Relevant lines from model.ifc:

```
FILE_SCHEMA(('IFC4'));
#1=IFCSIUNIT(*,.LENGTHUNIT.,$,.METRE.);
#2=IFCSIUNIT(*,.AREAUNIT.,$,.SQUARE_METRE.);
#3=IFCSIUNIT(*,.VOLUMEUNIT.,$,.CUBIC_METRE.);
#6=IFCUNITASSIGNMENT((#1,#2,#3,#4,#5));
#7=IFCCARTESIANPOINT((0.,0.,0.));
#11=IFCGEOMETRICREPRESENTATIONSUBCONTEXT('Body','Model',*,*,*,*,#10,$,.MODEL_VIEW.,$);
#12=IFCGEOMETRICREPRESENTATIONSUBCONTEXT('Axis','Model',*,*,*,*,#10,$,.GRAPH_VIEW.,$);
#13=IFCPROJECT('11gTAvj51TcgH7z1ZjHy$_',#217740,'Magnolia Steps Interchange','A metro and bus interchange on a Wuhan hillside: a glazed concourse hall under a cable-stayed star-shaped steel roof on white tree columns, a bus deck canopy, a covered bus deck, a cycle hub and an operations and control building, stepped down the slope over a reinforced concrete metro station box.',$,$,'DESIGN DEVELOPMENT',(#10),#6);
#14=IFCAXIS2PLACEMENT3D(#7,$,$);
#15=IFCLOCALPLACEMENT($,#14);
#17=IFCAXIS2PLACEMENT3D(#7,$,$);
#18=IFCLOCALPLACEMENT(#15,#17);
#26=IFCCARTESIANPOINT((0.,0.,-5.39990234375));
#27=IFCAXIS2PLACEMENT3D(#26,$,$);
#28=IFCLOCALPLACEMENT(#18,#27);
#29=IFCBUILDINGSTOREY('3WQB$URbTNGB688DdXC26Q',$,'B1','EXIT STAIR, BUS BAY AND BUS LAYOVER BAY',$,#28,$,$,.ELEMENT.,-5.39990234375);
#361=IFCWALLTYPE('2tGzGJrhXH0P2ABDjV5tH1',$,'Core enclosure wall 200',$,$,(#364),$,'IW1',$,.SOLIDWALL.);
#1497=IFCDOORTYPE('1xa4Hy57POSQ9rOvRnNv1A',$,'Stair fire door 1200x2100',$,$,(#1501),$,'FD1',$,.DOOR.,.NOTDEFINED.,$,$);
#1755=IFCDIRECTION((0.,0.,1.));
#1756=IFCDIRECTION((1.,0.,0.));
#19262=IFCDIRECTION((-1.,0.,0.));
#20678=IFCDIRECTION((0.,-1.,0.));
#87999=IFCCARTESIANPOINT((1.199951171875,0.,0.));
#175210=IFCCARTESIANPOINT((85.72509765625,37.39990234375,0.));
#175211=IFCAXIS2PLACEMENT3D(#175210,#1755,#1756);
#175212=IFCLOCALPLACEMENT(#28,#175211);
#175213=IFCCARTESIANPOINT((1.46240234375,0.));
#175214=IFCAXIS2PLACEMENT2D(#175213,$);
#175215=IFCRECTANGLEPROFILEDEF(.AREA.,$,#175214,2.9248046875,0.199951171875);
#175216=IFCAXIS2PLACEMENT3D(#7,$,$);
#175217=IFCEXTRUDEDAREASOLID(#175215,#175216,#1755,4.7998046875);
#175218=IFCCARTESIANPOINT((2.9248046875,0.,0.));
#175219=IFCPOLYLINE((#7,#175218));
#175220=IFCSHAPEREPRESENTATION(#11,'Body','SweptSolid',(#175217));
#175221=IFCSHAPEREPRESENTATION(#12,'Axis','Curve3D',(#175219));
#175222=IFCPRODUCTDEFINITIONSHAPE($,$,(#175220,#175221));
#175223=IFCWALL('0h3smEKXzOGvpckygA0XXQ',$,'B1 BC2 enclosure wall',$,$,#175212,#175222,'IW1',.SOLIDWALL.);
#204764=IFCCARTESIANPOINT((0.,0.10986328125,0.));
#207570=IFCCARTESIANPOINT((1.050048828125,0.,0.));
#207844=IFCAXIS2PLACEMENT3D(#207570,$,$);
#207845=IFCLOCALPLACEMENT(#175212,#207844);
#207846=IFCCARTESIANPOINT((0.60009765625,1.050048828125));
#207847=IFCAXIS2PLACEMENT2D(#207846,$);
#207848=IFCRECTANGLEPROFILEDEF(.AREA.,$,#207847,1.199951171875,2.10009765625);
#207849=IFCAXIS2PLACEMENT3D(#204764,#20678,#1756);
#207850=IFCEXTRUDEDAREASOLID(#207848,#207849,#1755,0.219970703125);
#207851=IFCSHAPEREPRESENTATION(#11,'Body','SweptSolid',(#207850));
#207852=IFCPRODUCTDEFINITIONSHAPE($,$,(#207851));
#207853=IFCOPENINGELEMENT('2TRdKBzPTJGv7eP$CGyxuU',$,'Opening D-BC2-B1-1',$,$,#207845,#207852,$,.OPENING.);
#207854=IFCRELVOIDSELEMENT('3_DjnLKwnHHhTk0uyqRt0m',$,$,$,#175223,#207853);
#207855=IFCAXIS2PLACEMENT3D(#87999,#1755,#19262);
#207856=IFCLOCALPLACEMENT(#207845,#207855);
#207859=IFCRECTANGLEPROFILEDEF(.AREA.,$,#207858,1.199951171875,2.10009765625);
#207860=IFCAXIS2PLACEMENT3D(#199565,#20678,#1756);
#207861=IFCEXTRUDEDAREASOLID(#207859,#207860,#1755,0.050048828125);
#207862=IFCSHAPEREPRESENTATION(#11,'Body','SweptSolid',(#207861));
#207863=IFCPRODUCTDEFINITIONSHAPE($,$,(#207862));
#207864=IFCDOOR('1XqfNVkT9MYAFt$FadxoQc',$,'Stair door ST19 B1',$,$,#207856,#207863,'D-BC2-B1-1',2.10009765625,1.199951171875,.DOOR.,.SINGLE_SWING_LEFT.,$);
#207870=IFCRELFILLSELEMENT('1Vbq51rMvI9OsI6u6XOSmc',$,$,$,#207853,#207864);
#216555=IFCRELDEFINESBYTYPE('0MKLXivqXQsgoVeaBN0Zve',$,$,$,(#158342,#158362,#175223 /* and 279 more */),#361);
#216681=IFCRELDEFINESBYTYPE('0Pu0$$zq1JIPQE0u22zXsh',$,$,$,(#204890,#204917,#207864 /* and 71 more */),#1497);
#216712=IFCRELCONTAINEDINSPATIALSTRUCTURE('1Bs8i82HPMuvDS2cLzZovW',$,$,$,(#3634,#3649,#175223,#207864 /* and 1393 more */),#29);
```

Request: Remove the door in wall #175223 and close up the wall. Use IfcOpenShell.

```python
import ifcopenshell
import ifcopenshell.api.feature
import ifcopenshell.api.root
import ifcopenshell.geom
import ifcopenshell.util.shape

model = ifcopenshell.open("model.ifc")
settings = ifcopenshell.geom.settings()


def volume(element):
    """Net volume in cubic metres, openings subtracted."""
    shape = ifcopenshell.geom.create_shape(settings, element)
    return ifcopenshell.util.shape.get_volume(shape.geometry)


door = model.by_id(207864)
opening = door.FillsVoids[0].RelatingOpeningElement
wall = opening.VoidsElements[0].RelatingBuildingElement
before = volume(wall)

ifcopenshell.api.root.remove_product(model, product=door)
ifcopenshell.api.feature.remove_feature(model, feature=opening)

after = volume(wall)

print(f"wall volume {before:.3f} -> {after:.3f} m3")

model.write("model_updated.ifc")
```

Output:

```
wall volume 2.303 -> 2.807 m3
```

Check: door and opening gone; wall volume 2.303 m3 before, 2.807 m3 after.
